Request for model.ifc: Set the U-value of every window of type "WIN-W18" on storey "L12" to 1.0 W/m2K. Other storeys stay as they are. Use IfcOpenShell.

First a look at what the model holds.

```python
import ifcopenshell
import ifcopenshell.util.element

model = ifcopenshell.open("model.ifc")
print(model.schema)
storey = next(s for s in model.by_type("IfcBuildingStorey") if s.Name == "L12")
windows = [e for e in ifcopenshell.util.element.get_decomposition(storey) if e.is_a("IfcWindow")]
seen = {}
for e in windows:
    element_type = ifcopenshell.util.element.get_type(e)
    key = (element_type.Name if element_type != e and element_type else None, ifcopenshell.util.element.get_pset(e, "Pset_WindowCommon", "ThermalTransmittance"))
    seen[key] = seen.get(key, 0) + 1
for (name, value), count in sorted(seen.items(), key=str):
    print(count, "x", name, "|", value)
```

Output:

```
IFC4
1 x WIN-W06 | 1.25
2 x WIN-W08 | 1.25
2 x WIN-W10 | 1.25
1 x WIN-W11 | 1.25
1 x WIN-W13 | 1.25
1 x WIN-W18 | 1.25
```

```python
import ifcopenshell
import ifcopenshell.api.pset
import ifcopenshell.util.element

model = ifcopenshell.open("model.ifc")

storey = next(s for s in model.by_type("IfcBuildingStorey") if s.Name == "L12")
windows = [e for e in ifcopenshell.util.element.get_decomposition(storey) if e.is_a("IfcWindow")]

count = 0
for e in windows:
    element_type = ifcopenshell.util.element.get_type(e)
    if element_type in (None, e) or element_type.Name != "WIN-W18":
        continue
    # add_pset returns the element's existing set when there is one.
    pset = ifcopenshell.api.pset.add_pset(model, product=e, name="Pset_WindowCommon")
    ifcopenshell.api.pset.edit_pset(model, pset=pset, properties={"ThermalTransmittance": 1.0})
    count += 1

print(count, "windows updated")

model.write("model-out.ifc")
```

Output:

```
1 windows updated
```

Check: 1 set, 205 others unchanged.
